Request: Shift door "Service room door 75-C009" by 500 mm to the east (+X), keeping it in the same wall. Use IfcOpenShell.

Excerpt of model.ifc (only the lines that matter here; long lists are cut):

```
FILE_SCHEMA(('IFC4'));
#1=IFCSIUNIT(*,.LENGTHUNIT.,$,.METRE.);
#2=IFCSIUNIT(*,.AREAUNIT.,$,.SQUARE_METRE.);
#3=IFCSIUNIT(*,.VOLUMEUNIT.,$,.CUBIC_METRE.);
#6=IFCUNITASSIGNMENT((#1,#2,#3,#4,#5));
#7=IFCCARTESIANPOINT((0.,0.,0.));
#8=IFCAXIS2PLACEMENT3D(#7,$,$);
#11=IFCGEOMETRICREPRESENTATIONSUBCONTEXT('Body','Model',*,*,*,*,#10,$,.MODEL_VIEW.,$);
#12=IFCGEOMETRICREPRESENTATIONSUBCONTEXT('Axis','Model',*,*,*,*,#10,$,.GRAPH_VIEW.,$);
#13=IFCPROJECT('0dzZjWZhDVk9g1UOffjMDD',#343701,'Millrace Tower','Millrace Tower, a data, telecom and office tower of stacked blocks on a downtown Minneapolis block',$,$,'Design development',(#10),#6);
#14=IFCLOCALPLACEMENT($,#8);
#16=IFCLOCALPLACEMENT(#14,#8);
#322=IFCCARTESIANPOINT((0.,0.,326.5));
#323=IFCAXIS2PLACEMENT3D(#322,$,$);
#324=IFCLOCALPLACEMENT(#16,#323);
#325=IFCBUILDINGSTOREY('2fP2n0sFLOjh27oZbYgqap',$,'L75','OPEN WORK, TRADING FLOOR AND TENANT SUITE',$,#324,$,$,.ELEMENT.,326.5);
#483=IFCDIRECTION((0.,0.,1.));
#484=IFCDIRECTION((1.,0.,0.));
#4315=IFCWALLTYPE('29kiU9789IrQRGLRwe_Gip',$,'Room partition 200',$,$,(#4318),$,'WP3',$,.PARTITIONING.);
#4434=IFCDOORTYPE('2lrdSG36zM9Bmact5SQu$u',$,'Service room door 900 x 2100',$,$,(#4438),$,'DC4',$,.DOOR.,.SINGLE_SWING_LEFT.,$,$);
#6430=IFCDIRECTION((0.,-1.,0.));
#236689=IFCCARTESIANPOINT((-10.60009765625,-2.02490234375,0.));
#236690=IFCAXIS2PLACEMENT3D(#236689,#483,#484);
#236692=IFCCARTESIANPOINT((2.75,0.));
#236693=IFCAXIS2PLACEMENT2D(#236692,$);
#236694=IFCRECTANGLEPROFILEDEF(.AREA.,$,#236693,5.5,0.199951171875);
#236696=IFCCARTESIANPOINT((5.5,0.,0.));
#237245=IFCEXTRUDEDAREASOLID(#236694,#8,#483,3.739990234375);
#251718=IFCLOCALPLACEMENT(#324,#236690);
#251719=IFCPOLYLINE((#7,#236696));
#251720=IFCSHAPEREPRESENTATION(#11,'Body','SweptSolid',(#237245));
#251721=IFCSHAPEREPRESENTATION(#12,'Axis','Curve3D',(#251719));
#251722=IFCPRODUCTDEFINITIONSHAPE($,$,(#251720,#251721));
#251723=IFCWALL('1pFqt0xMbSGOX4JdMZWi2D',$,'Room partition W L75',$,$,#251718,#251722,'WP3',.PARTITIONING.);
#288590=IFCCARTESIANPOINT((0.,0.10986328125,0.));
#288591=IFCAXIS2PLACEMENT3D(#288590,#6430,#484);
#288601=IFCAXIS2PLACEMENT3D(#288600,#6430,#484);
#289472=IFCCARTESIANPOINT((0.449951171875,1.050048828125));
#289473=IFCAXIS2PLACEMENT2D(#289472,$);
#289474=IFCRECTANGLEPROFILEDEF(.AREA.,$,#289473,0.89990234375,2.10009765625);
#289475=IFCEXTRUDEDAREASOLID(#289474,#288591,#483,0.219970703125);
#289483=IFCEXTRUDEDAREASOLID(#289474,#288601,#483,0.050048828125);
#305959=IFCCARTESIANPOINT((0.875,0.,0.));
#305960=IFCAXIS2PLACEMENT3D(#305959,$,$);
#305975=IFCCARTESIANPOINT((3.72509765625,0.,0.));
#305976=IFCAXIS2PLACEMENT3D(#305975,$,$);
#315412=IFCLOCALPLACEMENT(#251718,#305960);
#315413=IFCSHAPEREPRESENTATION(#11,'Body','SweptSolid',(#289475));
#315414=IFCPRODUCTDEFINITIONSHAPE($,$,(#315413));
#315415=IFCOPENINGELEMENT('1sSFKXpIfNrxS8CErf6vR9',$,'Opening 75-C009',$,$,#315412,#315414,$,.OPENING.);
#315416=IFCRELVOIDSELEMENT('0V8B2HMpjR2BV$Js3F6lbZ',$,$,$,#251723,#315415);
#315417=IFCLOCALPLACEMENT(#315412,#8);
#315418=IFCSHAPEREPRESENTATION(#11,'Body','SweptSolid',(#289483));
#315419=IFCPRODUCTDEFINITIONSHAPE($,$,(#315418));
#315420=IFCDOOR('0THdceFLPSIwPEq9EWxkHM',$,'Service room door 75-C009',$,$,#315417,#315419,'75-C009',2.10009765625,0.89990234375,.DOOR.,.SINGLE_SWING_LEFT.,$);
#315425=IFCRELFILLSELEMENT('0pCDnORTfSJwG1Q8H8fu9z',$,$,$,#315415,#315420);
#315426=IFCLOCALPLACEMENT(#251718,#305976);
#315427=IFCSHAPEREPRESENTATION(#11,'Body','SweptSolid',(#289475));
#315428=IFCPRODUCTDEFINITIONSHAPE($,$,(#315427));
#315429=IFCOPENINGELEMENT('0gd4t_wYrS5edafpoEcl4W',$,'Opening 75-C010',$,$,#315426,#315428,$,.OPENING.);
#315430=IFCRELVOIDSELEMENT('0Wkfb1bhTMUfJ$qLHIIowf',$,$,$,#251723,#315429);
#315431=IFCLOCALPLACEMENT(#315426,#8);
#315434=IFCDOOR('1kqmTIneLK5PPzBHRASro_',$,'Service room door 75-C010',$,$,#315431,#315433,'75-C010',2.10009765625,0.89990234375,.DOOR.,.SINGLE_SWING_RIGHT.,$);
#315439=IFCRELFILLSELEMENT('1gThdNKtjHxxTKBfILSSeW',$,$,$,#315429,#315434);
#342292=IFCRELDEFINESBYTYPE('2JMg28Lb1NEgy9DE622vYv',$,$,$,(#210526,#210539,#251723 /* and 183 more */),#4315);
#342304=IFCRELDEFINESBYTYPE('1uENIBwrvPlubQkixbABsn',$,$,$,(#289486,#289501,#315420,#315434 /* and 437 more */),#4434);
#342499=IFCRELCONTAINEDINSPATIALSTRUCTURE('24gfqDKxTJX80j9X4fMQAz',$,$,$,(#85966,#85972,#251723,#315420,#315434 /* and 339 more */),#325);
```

```python
import ifcopenshell
import ifcopenshell.api.geometry
import ifcopenshell.util.placement

model = ifcopenshell.open("model.ifc")

door = model.by_guid("0THdceFLPSIwPEq9EWxkHM")
opening = door.FillsVoids[0].RelatingOpeningElement
wall = opening.VoidsElements[0].RelatingBuildingElement

wall_matrix = ifcopenshell.util.placement.get_local_placement(wall.ObjectPlacement)
shift = wall_matrix[:3, 0] * 0.5
before = ifcopenshell.util.placement.get_local_placement(door.ObjectPlacement)[:3, 3].copy()

# The door is placed relative to its opening, so it follows when the opening moves.
matrix = ifcopenshell.util.placement.get_local_placement(opening.ObjectPlacement)
matrix[:3, 3] += shift
ifcopenshell.api.geometry.edit_object_placement(
    model, product=opening, matrix=matrix, is_si=False, should_transform_children=True
)

after = ifcopenshell.util.placement.get_local_placement(door.ObjectPlacement)[:3, 3]
print("door moved by", (after - before).round(3) + 0.0)

model.write("model_updated.ifc")
```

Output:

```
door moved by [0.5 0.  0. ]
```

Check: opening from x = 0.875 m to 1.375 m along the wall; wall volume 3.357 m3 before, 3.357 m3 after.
